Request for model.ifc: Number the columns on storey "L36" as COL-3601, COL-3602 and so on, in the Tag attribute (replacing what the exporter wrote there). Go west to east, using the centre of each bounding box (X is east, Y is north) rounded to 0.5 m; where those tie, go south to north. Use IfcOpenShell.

First a look at what the model holds.

```python
import ifcopenshell
import ifcopenshell.util.element
import ifcopenshell.util.placement

model = ifcopenshell.open("model.ifc")
print(model.schema)
storey = next(s for s in model.by_type("IfcBuildingStorey") if s.Name == "L36")
columns = [e for e in ifcopenshell.util.element.get_decomposition(storey) if e.is_a("IfcColumn")]
for e in sorted(columns, key=lambda e: e.id()):
    origin = ifcopenshell.util.placement.get_local_placement(e.ObjectPlacement)[:3, 3]
    print(e.id(), e.Tag, e.Name, origin.round(2) + 0.0, sep=" | ")
```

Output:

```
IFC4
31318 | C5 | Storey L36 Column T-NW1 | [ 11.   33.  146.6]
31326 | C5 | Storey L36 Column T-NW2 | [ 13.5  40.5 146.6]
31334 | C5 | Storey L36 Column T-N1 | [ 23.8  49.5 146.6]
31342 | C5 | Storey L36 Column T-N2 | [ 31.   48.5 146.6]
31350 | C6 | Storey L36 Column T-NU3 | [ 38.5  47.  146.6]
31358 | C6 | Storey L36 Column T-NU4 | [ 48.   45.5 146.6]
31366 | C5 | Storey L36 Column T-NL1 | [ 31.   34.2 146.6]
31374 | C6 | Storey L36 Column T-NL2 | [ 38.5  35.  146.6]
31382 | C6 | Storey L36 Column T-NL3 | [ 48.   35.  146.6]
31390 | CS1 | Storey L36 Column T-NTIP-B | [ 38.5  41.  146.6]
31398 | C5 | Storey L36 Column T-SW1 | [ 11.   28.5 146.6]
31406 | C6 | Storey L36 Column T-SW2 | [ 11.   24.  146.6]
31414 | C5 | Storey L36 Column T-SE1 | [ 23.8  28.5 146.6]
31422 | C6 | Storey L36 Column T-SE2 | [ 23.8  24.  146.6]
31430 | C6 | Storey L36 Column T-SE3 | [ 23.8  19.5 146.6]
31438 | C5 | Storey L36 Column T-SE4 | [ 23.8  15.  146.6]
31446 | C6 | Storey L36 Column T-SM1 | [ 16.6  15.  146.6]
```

```python
import ifcopenshell
import ifcopenshell.geom
import ifcopenshell.util.element
import ifcopenshell.util.shape

model = ifcopenshell.open("model.ifc")
settings = ifcopenshell.geom.settings()
settings.set("use-world-coords", True)


def centre(element):
    shape = ifcopenshell.geom.create_shape(settings, element)
    return ifcopenshell.util.shape.get_bbox_centroid(shape.geometry)


storey = next(s for s in model.by_type("IfcBuildingStorey") if s.Name == "L36")
columns = [e for e in ifcopenshell.util.element.get_decomposition(storey) if e.is_a("IfcColumn")]

# Insertion points can sit at a corner or the storey origin, so sort by the geometry (in metres).
centres = {e: centre(e) for e in columns}
columns.sort(key=lambda e: (round(centres[e][0] / 0.5), centres[e][1]))

for i, e in enumerate(columns, start=1):
    number = f"COL-36{i:02d}"
    e.Tag = number
    print(e.id(), number)

model.write("model_rev.ifc")
```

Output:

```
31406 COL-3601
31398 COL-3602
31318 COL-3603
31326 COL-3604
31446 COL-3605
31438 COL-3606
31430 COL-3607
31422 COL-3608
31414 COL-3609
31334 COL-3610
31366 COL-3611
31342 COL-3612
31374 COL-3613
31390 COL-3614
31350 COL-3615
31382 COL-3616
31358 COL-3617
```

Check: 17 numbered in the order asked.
